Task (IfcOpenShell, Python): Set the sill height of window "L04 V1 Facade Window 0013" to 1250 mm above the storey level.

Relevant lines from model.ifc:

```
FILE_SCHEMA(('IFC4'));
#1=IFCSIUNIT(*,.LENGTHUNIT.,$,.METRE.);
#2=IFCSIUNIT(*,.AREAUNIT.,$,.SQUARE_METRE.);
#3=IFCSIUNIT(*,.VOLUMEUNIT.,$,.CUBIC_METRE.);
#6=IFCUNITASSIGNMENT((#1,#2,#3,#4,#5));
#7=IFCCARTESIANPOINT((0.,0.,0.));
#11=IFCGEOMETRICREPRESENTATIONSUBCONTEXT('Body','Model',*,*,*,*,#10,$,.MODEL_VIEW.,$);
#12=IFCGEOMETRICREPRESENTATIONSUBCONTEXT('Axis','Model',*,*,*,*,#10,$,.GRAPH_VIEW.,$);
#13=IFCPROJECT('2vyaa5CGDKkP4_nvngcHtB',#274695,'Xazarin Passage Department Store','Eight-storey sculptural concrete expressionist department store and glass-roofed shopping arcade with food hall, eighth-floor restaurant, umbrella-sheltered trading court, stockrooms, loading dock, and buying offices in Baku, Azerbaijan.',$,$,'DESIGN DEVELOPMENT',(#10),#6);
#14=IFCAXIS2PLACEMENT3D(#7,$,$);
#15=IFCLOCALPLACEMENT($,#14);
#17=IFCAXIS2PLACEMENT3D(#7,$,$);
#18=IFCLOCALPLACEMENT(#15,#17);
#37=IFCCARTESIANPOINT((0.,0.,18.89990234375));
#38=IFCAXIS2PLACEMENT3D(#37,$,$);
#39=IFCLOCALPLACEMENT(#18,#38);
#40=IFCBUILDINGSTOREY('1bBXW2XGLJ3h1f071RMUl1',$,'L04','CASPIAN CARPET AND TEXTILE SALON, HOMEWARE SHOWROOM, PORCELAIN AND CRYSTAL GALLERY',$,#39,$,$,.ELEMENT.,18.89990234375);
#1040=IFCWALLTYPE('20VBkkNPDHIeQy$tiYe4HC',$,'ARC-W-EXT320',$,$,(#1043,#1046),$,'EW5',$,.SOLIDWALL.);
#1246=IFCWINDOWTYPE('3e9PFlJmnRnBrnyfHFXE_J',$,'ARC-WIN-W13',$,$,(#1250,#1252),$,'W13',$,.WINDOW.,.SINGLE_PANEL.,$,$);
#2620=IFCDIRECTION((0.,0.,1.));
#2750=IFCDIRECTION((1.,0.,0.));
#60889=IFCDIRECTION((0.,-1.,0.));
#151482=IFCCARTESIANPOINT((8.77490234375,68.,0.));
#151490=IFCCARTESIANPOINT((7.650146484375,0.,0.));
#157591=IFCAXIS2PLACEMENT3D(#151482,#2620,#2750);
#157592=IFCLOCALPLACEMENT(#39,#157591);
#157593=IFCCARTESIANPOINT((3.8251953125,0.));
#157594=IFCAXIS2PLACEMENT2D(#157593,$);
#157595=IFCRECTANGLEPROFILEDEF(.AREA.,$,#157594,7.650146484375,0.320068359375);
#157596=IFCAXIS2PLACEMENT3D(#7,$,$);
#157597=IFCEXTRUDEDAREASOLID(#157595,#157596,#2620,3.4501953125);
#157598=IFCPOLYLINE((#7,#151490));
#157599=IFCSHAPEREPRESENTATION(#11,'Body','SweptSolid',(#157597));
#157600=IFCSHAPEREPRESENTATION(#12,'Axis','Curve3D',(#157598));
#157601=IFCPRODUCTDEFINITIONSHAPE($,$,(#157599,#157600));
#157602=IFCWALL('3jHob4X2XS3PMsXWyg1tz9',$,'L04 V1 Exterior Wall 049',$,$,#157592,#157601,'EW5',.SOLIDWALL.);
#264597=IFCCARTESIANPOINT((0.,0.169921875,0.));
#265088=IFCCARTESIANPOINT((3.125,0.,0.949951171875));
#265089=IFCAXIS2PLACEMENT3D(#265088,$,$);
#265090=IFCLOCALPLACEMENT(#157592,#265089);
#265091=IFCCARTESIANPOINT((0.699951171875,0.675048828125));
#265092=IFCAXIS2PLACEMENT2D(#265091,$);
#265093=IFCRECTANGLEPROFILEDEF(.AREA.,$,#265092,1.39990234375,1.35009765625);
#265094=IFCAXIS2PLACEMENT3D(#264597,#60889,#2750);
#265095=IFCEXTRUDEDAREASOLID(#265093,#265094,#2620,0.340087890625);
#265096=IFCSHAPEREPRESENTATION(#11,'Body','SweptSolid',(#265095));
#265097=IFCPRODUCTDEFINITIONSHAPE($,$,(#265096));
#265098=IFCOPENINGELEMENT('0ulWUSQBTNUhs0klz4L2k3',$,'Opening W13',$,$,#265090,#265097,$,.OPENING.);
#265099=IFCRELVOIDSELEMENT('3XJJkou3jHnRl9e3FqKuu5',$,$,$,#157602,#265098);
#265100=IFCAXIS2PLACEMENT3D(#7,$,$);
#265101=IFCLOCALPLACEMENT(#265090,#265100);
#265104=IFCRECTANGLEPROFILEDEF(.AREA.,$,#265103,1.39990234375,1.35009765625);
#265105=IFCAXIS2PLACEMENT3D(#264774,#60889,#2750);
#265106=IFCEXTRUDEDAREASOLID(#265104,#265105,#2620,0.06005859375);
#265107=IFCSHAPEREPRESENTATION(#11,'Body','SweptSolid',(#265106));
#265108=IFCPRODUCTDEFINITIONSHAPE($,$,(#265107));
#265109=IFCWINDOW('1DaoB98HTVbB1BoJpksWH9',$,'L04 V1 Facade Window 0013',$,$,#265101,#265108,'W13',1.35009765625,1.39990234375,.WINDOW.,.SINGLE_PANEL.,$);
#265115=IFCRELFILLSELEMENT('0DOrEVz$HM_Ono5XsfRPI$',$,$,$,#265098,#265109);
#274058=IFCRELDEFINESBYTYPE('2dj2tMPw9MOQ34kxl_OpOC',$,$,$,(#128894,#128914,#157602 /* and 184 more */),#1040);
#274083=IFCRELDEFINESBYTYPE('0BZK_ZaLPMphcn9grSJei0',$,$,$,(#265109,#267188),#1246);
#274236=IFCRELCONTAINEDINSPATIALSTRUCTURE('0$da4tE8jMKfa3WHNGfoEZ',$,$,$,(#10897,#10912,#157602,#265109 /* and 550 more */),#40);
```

```python
import numpy as np
import ifcopenshell
import ifcopenshell.api.geometry
import ifcopenshell.geom
import ifcopenshell.util.element
import ifcopenshell.util.placement
import ifcopenshell.util.shape
import ifcopenshell.util.unit

model = ifcopenshell.open("model.ifc")
unit_scale = ifcopenshell.util.unit.calculate_unit_scale(model)

window = model.by_guid("1DaoB98HTVbB1BoJpksWH9")
opening = window.FillsVoids[0].RelatingOpeningElement
storey = ifcopenshell.util.element.get_container(window, ifc_class="IfcBuildingStorey")
level = ifcopenshell.util.placement.get_local_placement(storey.ObjectPlacement)[2, 3]

# The opening's origin need not be at the sill, so measure its lowest point.
shape = ifcopenshell.geom.create_shape(ifcopenshell.geom.settings(), opening)
bottom = ifcopenshell.util.shape.get_shape_bottom_elevation(shape, shape.geometry) / unit_scale
dz = level + 1.25 / unit_scale - bottom

shift = np.array([0.0, 0.0, dz])
# The window is placed relative to its opening, so it follows when the opening moves.
matrix = ifcopenshell.util.placement.get_local_placement(opening.ObjectPlacement)
matrix[:3, 3] += shift
ifcopenshell.api.geometry.edit_object_placement(
    model, product=opening, matrix=matrix, is_si=False, should_transform_children=True
)

print(f"moved by {dz * unit_scale:+.3f} m")

model.write("model_v2.ifc")
```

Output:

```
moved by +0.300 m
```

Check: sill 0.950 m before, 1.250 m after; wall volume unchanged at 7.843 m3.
